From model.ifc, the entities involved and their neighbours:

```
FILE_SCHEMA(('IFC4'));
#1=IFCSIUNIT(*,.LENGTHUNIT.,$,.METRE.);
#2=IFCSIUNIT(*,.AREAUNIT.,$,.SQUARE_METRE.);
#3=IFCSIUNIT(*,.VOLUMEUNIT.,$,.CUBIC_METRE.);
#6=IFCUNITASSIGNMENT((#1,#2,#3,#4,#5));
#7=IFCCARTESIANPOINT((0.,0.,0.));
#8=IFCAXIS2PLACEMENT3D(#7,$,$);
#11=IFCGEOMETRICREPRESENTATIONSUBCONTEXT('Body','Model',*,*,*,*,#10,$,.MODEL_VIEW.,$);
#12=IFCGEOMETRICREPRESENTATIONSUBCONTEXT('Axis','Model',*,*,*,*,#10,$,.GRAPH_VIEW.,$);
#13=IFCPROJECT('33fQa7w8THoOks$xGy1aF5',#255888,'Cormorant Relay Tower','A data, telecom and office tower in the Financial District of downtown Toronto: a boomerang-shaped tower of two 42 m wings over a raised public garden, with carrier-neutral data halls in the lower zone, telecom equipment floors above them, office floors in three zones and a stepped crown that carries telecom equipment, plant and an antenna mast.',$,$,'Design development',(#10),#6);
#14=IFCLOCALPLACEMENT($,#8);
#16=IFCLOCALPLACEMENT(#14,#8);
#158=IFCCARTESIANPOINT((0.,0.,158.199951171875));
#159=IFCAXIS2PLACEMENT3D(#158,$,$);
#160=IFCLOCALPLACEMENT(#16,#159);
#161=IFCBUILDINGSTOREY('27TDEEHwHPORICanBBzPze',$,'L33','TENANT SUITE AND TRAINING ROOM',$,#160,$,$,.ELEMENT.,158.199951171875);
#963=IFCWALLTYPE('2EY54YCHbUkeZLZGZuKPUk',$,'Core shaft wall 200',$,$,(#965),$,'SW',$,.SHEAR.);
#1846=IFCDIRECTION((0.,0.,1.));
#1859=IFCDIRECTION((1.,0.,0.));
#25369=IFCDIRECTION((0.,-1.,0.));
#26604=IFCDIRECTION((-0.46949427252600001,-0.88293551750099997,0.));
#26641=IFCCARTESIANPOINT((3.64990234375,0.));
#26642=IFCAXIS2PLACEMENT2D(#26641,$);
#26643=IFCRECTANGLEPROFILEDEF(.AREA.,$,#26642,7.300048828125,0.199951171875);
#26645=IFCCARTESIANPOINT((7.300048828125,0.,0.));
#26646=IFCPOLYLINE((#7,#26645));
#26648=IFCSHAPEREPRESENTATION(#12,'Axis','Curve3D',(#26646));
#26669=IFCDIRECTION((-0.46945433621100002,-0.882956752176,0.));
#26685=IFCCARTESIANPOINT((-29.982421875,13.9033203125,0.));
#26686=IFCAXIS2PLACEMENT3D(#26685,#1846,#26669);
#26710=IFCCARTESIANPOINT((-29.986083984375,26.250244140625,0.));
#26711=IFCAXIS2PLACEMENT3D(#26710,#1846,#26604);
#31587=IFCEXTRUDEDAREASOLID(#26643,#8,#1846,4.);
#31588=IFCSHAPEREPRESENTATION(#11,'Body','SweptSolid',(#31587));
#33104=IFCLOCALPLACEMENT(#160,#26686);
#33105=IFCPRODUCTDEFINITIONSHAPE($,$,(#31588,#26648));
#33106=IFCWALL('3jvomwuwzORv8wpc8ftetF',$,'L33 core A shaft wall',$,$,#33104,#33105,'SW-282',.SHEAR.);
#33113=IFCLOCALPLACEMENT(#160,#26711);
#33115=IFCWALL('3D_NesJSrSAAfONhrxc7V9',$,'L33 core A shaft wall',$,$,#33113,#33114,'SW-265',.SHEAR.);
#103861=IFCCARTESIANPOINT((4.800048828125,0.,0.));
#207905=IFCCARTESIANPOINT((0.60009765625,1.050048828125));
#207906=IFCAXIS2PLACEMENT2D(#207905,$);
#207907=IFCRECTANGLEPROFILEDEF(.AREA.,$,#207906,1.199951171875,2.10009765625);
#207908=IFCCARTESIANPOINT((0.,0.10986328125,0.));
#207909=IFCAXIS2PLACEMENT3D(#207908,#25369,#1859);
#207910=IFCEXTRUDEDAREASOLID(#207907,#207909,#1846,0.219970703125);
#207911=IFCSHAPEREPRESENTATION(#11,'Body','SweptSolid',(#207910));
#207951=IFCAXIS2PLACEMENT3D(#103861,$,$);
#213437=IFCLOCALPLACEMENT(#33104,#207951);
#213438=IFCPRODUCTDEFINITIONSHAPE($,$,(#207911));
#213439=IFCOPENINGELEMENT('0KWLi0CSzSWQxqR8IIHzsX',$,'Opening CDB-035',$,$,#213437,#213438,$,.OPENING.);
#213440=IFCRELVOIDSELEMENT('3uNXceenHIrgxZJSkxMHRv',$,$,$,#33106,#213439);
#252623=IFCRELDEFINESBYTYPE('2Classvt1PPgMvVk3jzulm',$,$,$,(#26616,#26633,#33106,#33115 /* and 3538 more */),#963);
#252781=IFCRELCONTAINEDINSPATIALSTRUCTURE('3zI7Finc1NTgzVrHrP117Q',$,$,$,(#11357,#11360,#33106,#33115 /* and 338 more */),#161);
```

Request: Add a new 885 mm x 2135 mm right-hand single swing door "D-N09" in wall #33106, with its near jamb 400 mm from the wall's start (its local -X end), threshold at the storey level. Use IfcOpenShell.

```python
import numpy as np
import ifcopenshell
import ifcopenshell.api.feature
import ifcopenshell.api.geometry
import ifcopenshell.api.root
import ifcopenshell.api.spatial
import ifcopenshell.geom
import ifcopenshell.util.element
import ifcopenshell.util.placement
import ifcopenshell.util.representation
import ifcopenshell.util.shape
import ifcopenshell.util.unit

model = ifcopenshell.open("model.ifc")
unit_scale = ifcopenshell.util.unit.calculate_unit_scale(model)
settings = ifcopenshell.geom.settings()


def volume(element):
    """Net volume in cubic metres, openings subtracted."""
    shape = ifcopenshell.geom.create_shape(settings, element)
    return ifcopenshell.util.shape.get_volume(shape.geometry)


wall = model.by_id(33106)
storey = ifcopenshell.util.element.get_container(wall, ifc_class="IfcBuildingStorey")
context = ifcopenshell.util.representation.get_context(model, "Model", "Body", "MODEL_VIEW")
before = volume(wall)

width, height, from_end, sill = 0.885, 2.135, 0.4, 0.0  # metres

# The wall runs along its own X axis, and the end named is its -X end.
wall_shape = ifcopenshell.geom.create_shape(settings, wall)
x, y, z = ifcopenshell.util.shape.get_vertices(wall_shape.geometry).T
start = x.min() + from_end
face, thickness = float(y.min()), float(y.max() - y.min())
wall_matrix = ifcopenshell.util.placement.get_local_placement(wall.ObjectPlacement)
level = ifcopenshell.util.placement.get_local_placement(storey.ObjectPlacement)[2, 3]


def in_wall(x, y):
    """Placement at x, y metres in the wall's axes, at sill height."""
    matrix = wall_matrix.copy()
    matrix[:, 3] = wall_matrix @ np.array([x / unit_scale, y / unit_scale, 0.0, 1.0])
    matrix[2, 3] = level + sill / unit_scale
    return matrix


# Opening: a box that overshoots both wall faces by 50 mm.
opening = ifcopenshell.api.root.create_entity(model, ifc_class="IfcOpeningElement", predefined_type="OPENING")
box = ifcopenshell.api.geometry.add_wall_representation(
    model, context=context, length=width, height=height, thickness=thickness + 0.1
)
ifcopenshell.api.geometry.assign_representation(model, product=opening, representation=box)
ifcopenshell.api.geometry.edit_object_placement(model, product=opening, matrix=in_wall(start, face - 0.05), is_si=False)
ifcopenshell.api.feature.add_feature(model, feature=opening, element=wall)

door = ifcopenshell.api.root.create_entity(model, ifc_class="IfcDoor", name="D-N09", predefined_type="DOOR")
door.OverallWidth, door.OverallHeight = width / unit_scale, height / unit_scale
door.OperationType = "SINGLE_SWING_RIGHT"
body = ifcopenshell.api.geometry.add_door_representation(
    model,
    context=context,
    overall_width=door.OverallWidth,
    overall_height=door.OverallHeight,
    operation_type="SINGLE_SWING_RIGHT",
    lining_properties={"LiningDepth": thickness / unit_scale, "ThresholdDepth": thickness / unit_scale},
)
ifcopenshell.api.geometry.assign_representation(model, product=door, representation=body)
ifcopenshell.api.spatial.assign_container(model, products=[door], relating_structure=storey)
ifcopenshell.api.feature.add_filling(model, opening=opening, element=door)

# The lining spans the wall, so the door starts at the wall face.
ifcopenshell.api.geometry.edit_object_placement(model, product=door, matrix=in_wall(start, face), is_si=False)

after = volume(wall)

print(f"wall volume {before:.3f} -> {after:.3f} m3")

model.write("model_v2.ifc")
```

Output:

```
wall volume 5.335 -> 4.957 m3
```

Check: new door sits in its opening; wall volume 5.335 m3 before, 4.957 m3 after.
